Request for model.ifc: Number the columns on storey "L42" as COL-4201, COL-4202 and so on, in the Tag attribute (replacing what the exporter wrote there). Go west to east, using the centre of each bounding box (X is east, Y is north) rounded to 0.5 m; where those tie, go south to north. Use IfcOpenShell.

First a look at what the model holds.

```python
import ifcopenshell
import ifcopenshell.util.element
import ifcopenshell.util.placement

model = ifcopenshell.open("model.ifc")
print(model.schema)
storey = next(s for s in model.by_type("IfcBuildingStorey") if s.Name == "L42")
columns = [e for e in ifcopenshell.util.element.get_decomposition(storey) if e.is_a("IfcColumn")]
for e in sorted(columns, key=lambda e: e.id()):
    origin = ifcopenshell.util.placement.get_local_placement(e.ObjectPlacement)[:3, 3]
    print(e.id(), e.Tag, e.Name, origin.round(2) + 0.0, sep=" | ")
```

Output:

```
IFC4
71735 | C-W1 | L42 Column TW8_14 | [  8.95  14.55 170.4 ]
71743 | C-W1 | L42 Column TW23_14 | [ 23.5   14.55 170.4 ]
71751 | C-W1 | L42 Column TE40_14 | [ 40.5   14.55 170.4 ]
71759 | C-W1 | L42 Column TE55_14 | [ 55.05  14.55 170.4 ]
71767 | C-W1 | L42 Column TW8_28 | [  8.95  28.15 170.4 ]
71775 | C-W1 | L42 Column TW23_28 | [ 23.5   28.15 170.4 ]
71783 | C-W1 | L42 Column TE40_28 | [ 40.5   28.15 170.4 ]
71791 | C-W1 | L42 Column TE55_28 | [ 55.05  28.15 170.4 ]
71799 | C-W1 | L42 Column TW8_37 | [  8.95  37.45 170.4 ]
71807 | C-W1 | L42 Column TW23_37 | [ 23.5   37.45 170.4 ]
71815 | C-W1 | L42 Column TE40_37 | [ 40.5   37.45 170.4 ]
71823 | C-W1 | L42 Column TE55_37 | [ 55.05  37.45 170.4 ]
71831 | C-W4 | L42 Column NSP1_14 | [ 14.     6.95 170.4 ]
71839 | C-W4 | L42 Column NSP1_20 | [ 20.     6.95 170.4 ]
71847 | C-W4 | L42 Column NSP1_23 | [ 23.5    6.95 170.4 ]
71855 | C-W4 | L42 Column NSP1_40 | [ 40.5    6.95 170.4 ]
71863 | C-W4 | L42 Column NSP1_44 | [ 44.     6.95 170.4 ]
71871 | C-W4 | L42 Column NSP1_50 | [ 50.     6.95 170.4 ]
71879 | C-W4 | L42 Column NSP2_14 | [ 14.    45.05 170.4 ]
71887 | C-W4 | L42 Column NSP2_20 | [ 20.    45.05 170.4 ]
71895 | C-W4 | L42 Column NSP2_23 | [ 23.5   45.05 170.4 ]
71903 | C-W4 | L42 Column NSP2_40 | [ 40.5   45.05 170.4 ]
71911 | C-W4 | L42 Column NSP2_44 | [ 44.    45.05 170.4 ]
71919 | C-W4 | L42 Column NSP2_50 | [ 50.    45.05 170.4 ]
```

```python
import ifcopenshell
import ifcopenshell.geom
import ifcopenshell.util.element
import ifcopenshell.util.shape

model = ifcopenshell.open("model.ifc")
settings = ifcopenshell.geom.settings()
settings.set("use-world-coords", True)


def centre(element):
    shape = ifcopenshell.geom.create_shape(settings, element)
    return ifcopenshell.util.shape.get_bbox_centroid(shape.geometry)


storey = next(s for s in model.by_type("IfcBuildingStorey") if s.Name == "L42")
columns = [e for e in ifcopenshell.util.element.get_decomposition(storey) if e.is_a("IfcColumn")]

# Insertion points can sit at a corner or the storey origin, so sort by the geometry (in metres).
centres = {e: centre(e) for e in columns}
columns.sort(key=lambda e: (round(centres[e][0] / 0.5), centres[e][1]))

for i, e in enumerate(columns, start=1):
    number = f"COL-42{i:02d}"
    e.Tag = number
    print(e.id(), number)

model.write("model-out.ifc")
```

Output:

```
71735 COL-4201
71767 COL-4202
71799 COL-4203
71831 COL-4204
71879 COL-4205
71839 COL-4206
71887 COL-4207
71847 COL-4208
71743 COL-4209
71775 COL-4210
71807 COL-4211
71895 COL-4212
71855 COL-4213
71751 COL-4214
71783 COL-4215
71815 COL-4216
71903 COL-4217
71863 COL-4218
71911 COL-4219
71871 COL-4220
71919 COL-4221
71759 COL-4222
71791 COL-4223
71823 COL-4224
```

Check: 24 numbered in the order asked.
